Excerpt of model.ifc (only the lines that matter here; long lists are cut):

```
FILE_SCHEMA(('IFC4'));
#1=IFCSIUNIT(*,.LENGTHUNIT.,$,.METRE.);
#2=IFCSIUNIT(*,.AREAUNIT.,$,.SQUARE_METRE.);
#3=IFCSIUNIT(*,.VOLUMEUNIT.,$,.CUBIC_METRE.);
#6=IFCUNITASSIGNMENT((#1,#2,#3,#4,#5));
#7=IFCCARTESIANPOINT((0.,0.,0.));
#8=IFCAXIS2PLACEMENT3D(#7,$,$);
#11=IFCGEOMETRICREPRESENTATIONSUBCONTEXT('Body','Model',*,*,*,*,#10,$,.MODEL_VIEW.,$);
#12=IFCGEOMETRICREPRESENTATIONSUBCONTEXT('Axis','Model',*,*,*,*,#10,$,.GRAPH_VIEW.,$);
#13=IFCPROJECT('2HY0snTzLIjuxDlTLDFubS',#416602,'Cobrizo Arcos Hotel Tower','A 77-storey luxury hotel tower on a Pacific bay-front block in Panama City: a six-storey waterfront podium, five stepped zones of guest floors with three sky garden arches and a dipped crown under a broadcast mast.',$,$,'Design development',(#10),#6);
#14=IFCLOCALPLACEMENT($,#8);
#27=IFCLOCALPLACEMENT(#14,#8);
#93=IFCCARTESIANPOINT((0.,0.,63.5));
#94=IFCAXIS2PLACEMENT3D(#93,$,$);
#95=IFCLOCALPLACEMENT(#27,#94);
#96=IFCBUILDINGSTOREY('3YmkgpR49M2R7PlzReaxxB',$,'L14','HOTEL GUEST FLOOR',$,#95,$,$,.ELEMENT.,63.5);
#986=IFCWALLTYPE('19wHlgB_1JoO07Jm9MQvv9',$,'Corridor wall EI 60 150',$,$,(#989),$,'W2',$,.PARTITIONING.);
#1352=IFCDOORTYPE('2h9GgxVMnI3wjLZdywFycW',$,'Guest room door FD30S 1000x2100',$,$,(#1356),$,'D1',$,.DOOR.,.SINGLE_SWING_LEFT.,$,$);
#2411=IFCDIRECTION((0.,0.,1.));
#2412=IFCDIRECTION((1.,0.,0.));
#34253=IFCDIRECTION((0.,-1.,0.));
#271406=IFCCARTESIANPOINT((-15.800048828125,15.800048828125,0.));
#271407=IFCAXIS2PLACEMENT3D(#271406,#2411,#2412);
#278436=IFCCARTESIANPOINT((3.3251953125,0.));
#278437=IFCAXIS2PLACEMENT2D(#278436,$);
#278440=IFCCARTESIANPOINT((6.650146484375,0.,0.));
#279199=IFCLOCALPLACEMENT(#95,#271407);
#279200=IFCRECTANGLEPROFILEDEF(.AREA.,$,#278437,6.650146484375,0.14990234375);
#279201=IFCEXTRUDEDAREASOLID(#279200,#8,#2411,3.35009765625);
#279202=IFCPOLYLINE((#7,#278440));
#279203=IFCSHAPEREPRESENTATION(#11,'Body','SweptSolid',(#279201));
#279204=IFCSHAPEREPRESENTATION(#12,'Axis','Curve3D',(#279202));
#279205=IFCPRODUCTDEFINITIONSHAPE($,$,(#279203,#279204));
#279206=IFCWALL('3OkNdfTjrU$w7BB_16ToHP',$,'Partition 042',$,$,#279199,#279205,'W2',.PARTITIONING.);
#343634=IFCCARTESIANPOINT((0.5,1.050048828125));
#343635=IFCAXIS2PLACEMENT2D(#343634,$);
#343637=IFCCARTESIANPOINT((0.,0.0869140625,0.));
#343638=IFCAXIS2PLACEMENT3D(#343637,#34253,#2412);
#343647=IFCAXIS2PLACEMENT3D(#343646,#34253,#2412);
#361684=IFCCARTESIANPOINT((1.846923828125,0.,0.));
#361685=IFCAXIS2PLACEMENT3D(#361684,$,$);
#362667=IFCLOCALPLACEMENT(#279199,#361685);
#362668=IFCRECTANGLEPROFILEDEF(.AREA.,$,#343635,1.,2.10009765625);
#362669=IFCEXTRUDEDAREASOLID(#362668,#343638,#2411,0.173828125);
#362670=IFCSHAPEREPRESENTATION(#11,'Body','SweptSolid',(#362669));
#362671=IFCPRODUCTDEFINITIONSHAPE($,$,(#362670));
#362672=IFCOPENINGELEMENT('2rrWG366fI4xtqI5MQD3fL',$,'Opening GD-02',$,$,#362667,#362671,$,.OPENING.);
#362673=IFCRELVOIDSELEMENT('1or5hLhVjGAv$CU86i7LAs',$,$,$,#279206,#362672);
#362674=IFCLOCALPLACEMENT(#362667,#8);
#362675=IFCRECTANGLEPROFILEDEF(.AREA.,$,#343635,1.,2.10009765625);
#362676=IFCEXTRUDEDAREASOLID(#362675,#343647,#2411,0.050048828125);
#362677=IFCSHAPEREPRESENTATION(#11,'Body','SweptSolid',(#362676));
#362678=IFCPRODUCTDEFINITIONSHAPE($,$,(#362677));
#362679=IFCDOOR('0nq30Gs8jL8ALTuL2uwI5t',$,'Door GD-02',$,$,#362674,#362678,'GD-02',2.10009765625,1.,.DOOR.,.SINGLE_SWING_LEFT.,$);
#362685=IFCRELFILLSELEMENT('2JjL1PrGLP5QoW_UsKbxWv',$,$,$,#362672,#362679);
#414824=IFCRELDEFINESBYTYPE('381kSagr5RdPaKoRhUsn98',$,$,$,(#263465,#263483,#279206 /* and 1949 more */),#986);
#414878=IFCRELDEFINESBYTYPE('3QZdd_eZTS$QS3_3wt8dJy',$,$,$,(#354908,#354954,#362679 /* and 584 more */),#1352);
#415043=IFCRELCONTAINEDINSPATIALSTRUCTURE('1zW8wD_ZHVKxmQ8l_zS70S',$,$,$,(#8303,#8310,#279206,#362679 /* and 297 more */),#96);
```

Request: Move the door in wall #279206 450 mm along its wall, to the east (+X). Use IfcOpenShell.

```python
import ifcopenshell
import ifcopenshell.api.geometry
import ifcopenshell.util.placement

model = ifcopenshell.open("model.ifc")

door = model.by_id(362679)
opening = door.FillsVoids[0].RelatingOpeningElement
wall = opening.VoidsElements[0].RelatingBuildingElement

wall_matrix = ifcopenshell.util.placement.get_local_placement(wall.ObjectPlacement)
shift = wall_matrix[:3, 0] * 0.45
before = ifcopenshell.util.placement.get_local_placement(door.ObjectPlacement)[:3, 3].copy()

# The door is placed relative to its opening, so it follows when the opening moves.
matrix = ifcopenshell.util.placement.get_local_placement(opening.ObjectPlacement)
matrix[:3, 3] += shift
ifcopenshell.api.geometry.edit_object_placement(
    model, product=opening, matrix=matrix, is_si=False, should_transform_children=True
)

after = ifcopenshell.util.placement.get_local_placement(door.ObjectPlacement)[:3, 3]
print("door moved by", (after - before).round(3) + 0.0)

model.write("model-out.ifc")
```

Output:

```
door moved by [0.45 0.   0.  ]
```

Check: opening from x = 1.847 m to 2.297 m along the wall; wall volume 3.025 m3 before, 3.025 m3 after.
